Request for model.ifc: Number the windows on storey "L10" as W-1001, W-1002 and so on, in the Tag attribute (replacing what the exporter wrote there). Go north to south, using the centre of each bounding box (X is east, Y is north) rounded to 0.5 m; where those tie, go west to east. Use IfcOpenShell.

First a look at what the model holds.

```python
import ifcopenshell
import ifcopenshell.util.element
import ifcopenshell.util.placement

model = ifcopenshell.open("model.ifc")
print(model.schema)
storey = next(s for s in model.by_type("IfcBuildingStorey") if s.Name == "L10")
windows = [e for e in ifcopenshell.util.element.get_decomposition(storey) if e.is_a("IfcWindow")]
for e in sorted(windows, key=lambda e: e.id()):
    origin = ifcopenshell.util.placement.get_local_placement(e.ObjectPlacement)[:3, 3]
    print(e.id(), e.Tag, e.Name, origin.round(2) + 0.0, sep=" | ")
```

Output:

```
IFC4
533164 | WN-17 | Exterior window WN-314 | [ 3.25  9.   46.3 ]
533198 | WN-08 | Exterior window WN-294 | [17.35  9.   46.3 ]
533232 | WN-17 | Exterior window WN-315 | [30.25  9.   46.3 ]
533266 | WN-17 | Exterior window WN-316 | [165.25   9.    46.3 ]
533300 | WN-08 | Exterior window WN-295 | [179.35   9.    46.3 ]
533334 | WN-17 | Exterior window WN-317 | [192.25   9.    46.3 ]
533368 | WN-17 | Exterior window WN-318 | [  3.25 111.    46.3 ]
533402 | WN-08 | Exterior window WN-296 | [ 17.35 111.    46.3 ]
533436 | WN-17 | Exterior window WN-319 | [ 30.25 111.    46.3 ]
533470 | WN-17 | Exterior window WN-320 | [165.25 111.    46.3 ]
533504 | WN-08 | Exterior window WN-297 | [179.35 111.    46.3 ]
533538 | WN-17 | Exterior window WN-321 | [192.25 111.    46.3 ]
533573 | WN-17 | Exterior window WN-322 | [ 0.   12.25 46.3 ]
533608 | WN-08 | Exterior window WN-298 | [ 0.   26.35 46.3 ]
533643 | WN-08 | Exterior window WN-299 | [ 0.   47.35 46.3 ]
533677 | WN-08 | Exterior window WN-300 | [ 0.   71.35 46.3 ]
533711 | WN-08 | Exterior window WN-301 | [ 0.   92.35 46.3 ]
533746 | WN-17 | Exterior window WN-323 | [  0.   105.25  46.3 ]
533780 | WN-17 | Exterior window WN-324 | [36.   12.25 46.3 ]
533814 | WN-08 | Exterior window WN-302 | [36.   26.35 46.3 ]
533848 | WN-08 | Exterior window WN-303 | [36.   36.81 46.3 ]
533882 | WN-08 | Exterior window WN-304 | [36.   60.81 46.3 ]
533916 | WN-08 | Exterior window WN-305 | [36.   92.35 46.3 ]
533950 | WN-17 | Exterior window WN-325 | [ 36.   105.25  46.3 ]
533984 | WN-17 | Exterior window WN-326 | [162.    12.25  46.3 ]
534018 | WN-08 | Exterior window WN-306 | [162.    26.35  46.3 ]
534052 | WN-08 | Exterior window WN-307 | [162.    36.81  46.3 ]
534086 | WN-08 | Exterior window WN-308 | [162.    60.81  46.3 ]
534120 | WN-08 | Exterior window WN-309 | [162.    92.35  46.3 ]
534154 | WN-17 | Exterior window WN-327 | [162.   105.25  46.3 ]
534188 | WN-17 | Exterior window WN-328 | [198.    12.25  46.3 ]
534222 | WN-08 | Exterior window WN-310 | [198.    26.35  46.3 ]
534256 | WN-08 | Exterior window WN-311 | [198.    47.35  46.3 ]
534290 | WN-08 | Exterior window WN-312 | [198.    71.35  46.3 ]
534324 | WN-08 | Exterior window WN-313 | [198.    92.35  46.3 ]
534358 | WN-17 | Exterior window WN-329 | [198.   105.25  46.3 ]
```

```python
import ifcopenshell
import ifcopenshell.geom
import ifcopenshell.util.element
import ifcopenshell.util.shape

model = ifcopenshell.open("model.ifc")
settings = ifcopenshell.geom.settings()
settings.set("use-world-coords", True)


def centre(element):
    shape = ifcopenshell.geom.create_shape(settings, element)
    return ifcopenshell.util.shape.get_bbox_centroid(shape.geometry)


storey = next(s for s in model.by_type("IfcBuildingStorey") if s.Name == "L10")
windows = [e for e in ifcopenshell.util.element.get_decomposition(storey) if e.is_a("IfcWindow")]

# Insertion points can sit at a corner or the storey origin, so sort by the geometry (in metres).
centres = {e: centre(e) for e in windows}
windows.sort(key=lambda e: (-round(centres[e][1] / 0.5), centres[e][0]))

for i, e in enumerate(windows, start=1):
    number = f"W-10{i:02d}"
    e.Tag = number
    print(e.id(), number)

model.write("model_updated.ifc")
```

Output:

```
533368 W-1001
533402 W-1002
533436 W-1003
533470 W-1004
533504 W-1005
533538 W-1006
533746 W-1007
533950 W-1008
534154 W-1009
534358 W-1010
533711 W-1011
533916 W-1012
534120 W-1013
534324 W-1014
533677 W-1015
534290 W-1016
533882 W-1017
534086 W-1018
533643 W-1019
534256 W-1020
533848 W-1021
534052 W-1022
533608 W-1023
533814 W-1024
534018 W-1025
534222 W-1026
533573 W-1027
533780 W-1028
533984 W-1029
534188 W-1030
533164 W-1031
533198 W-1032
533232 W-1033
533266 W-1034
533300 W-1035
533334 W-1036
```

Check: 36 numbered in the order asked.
